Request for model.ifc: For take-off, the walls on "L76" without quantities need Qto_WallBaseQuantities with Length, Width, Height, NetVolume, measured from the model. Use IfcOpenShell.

First a look at what the model holds.

```python
import ifcopenshell
import ifcopenshell.util.element
import ifcopenshell.util.unit

model = ifcopenshell.open("model.ifc")
print(model.schema)
for unit_type in ("LENGTHUNIT", "AREAUNIT", "VOLUMEUNIT"):
    print(unit_type, ifcopenshell.util.unit.calculate_unit_scale(model, unit_type))
storey = next(s for s in model.by_type("IfcBuildingStorey") if s.Name == "L76")
walls = [e for e in ifcopenshell.util.element.get_decomposition(storey) if e.is_a("IfcWall")]
for e in sorted(walls, key=lambda e: e.id()):
    print(e.id(), e.is_a(), e.Name, list(ifcopenshell.util.element.get_psets(e, qtos_only=True)), sep=" | ")
```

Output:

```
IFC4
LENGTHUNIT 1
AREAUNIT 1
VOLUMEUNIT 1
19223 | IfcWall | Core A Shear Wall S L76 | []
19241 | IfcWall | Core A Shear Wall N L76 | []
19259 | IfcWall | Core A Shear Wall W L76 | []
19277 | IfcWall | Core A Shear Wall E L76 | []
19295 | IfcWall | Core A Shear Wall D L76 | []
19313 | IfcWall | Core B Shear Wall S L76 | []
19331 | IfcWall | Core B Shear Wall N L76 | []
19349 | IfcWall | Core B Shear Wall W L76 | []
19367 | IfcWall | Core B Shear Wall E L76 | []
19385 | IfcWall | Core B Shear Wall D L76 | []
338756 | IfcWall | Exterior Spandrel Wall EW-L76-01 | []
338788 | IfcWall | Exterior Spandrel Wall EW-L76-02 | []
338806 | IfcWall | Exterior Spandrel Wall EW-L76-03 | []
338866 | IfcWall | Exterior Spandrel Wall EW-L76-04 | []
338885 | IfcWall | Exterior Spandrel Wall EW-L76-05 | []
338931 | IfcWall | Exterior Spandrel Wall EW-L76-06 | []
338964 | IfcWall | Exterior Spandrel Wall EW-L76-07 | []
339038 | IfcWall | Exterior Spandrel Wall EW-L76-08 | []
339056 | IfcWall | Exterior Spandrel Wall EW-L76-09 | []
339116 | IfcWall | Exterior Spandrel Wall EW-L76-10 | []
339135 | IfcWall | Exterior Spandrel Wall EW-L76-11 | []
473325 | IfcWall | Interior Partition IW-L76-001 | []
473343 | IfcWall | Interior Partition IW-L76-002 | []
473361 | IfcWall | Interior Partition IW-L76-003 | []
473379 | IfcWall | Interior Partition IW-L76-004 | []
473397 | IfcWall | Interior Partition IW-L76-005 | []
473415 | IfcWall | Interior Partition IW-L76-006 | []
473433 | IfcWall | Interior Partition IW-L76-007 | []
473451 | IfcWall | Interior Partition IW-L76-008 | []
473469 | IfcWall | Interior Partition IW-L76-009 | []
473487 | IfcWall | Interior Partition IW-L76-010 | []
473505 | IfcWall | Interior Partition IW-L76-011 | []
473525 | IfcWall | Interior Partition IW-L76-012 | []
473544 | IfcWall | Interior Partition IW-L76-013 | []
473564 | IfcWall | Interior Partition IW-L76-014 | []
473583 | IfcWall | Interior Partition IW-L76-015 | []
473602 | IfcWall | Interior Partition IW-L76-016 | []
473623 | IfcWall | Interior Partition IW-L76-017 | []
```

```python
import ifcopenshell
import ifcopenshell.api.pset
import ifcopenshell.geom
import ifcopenshell.util.element
import ifcopenshell.util.shape
import ifcopenshell.util.unit

model = ifcopenshell.open("model.ifc")
unit_scale = ifcopenshell.util.unit.calculate_unit_scale(model)
volume_scale = ifcopenshell.util.unit.calculate_unit_scale(model, "VOLUMEUNIT")
settings = ifcopenshell.geom.settings()

storey = next(s for s in model.by_type("IfcBuildingStorey") if s.Name == "L76")
walls = [e for e in ifcopenshell.util.element.get_decomposition(storey) if e.is_a("IfcWall")]

for e in sorted(walls, key=lambda e: e.id()):
    if ifcopenshell.util.element.get_psets(e, qtos_only=True, should_inherit=False):
        continue
    # Geometry comes back in metres, in the element's own axes.
    shape = ifcopenshell.geom.create_shape(settings, e)
    values = {
        "Length": ifcopenshell.util.shape.get_x(shape.geometry) / unit_scale,
        "Width": ifcopenshell.util.shape.get_y(shape.geometry) / unit_scale,
        "Height": ifcopenshell.util.shape.get_z(shape.geometry) / unit_scale,
        "NetVolume": ifcopenshell.util.shape.get_volume(shape.geometry) / volume_scale,
    }
    qto = ifcopenshell.api.pset.add_qto(model, product=e, name="Qto_WallBaseQuantities")
    ifcopenshell.api.pset.edit_qto(model, qto=qto, properties=values)
    print(e.id(), {k: round(v, 3) for k, v in values.items()})

model.write("model-out.ifc")
```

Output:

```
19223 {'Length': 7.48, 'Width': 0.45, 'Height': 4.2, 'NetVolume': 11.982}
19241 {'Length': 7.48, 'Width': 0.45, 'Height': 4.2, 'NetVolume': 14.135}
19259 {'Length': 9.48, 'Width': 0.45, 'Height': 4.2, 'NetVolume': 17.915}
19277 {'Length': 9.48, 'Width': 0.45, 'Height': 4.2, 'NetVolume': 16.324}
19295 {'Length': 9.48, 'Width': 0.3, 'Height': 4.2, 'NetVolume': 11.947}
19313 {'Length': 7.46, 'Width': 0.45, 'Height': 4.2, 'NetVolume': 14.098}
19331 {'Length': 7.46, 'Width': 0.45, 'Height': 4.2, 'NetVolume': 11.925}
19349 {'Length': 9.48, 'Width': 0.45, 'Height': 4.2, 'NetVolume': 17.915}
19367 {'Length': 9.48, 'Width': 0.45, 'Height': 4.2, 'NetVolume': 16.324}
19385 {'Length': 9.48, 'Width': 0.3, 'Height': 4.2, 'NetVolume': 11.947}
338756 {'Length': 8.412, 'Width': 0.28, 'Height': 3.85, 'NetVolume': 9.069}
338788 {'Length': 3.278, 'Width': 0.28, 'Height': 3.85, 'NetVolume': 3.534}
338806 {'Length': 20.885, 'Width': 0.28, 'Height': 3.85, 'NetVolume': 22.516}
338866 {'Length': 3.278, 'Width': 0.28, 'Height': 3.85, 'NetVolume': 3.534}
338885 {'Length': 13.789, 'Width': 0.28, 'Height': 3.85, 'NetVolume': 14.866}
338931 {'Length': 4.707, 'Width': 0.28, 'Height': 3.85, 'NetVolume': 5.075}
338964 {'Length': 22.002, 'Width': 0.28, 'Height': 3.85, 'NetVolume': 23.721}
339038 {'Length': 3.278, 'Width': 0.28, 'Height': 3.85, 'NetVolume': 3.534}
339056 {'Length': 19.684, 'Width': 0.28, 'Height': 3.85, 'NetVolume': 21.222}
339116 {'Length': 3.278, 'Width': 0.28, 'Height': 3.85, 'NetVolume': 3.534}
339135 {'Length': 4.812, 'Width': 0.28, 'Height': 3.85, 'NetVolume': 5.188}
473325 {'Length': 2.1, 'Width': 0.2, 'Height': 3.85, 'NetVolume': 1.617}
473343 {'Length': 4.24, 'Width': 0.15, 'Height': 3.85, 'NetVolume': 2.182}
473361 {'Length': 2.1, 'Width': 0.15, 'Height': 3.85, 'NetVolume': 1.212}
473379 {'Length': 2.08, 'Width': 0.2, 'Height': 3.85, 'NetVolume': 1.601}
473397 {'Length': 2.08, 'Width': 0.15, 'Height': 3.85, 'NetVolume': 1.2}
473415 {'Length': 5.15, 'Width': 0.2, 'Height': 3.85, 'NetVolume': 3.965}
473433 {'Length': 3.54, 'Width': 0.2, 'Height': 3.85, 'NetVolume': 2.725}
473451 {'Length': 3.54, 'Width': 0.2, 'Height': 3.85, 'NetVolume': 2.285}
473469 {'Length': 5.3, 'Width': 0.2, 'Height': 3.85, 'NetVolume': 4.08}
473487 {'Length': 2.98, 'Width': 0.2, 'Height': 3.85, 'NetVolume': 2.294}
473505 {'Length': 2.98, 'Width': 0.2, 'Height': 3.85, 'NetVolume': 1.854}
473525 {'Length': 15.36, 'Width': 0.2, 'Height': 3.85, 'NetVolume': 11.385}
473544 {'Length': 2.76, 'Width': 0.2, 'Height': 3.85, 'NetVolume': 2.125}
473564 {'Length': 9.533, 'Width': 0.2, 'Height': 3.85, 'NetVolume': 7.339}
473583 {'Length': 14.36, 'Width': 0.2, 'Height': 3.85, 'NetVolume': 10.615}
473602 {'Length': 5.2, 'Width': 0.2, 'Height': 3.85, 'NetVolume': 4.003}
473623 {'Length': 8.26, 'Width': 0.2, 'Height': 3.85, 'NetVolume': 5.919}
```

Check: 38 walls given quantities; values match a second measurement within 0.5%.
